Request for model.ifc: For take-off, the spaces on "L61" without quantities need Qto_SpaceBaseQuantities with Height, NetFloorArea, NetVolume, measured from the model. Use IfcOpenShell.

First a look at what the model holds.

```python
import ifcopenshell
import ifcopenshell.util.element
import ifcopenshell.util.unit

model = ifcopenshell.open("model.ifc")
print(model.schema)
for unit_type in ("LENGTHUNIT", "AREAUNIT", "VOLUMEUNIT"):
    print(unit_type, ifcopenshell.util.unit.calculate_unit_scale(model, unit_type))
storey = next(s for s in model.by_type("IfcBuildingStorey") if s.Name == "L61")
spaces = [e for e in ifcopenshell.util.element.get_decomposition(storey) if e.is_a("IfcSpace")]
for e in sorted(spaces, key=lambda e: e.id()):
    print(e.id(), e.is_a(), e.Name, list(ifcopenshell.util.element.get_psets(e, qtos_only=True)), sep=" | ")
```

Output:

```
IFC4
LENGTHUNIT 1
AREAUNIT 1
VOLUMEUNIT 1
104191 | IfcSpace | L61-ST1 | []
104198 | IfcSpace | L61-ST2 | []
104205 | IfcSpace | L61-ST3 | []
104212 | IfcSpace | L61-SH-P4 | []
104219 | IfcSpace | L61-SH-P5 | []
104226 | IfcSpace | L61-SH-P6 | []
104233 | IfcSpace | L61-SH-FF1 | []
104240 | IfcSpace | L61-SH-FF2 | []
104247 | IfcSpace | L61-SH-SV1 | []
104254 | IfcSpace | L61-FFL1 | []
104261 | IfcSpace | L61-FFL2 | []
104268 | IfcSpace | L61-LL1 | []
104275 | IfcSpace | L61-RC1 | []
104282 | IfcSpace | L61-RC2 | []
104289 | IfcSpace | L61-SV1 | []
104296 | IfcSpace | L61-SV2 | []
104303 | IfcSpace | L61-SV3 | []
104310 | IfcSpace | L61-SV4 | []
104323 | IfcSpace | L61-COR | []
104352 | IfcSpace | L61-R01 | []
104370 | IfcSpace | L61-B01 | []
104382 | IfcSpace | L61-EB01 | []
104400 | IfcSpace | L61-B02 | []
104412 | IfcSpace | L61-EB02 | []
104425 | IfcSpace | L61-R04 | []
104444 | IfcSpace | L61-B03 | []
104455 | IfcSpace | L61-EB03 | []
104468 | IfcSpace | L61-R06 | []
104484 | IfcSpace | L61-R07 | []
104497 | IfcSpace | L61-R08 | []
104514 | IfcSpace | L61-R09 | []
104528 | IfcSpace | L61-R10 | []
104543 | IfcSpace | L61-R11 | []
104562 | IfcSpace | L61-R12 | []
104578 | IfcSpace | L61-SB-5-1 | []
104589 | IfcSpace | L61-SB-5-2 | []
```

```python
import ifcopenshell
import ifcopenshell.api.pset
import ifcopenshell.geom
import ifcopenshell.util.element
import ifcopenshell.util.shape
import ifcopenshell.util.unit

model = ifcopenshell.open("model.ifc")
unit_scale = ifcopenshell.util.unit.calculate_unit_scale(model)
area_scale = ifcopenshell.util.unit.calculate_unit_scale(model, "AREAUNIT")
volume_scale = ifcopenshell.util.unit.calculate_unit_scale(model, "VOLUMEUNIT")
settings = ifcopenshell.geom.settings()

storey = next(s for s in model.by_type("IfcBuildingStorey") if s.Name == "L61")
spaces = [e for e in ifcopenshell.util.element.get_decomposition(storey) if e.is_a("IfcSpace")]

for e in sorted(spaces, key=lambda e: e.id()):
    if ifcopenshell.util.element.get_psets(e, qtos_only=True, should_inherit=False):
        continue
    # Geometry comes back in metres, in the element's own axes.
    shape = ifcopenshell.geom.create_shape(settings, e)
    values = {
        "Height": ifcopenshell.util.shape.get_z(shape.geometry) / unit_scale,
        "NetFloorArea": ifcopenshell.util.shape.get_footprint_area(shape.geometry) / area_scale,
        "NetVolume": ifcopenshell.util.shape.get_volume(shape.geometry) / volume_scale,
    }
    qto = ifcopenshell.api.pset.add_qto(model, product=e, name="Qto_SpaceBaseQuantities")
    ifcopenshell.api.pset.edit_qto(model, qto=qto, properties=values)
    print(e.id(), {k: round(v, 3) for k, v in values.items()})

model.write("model_edited.ifc")
```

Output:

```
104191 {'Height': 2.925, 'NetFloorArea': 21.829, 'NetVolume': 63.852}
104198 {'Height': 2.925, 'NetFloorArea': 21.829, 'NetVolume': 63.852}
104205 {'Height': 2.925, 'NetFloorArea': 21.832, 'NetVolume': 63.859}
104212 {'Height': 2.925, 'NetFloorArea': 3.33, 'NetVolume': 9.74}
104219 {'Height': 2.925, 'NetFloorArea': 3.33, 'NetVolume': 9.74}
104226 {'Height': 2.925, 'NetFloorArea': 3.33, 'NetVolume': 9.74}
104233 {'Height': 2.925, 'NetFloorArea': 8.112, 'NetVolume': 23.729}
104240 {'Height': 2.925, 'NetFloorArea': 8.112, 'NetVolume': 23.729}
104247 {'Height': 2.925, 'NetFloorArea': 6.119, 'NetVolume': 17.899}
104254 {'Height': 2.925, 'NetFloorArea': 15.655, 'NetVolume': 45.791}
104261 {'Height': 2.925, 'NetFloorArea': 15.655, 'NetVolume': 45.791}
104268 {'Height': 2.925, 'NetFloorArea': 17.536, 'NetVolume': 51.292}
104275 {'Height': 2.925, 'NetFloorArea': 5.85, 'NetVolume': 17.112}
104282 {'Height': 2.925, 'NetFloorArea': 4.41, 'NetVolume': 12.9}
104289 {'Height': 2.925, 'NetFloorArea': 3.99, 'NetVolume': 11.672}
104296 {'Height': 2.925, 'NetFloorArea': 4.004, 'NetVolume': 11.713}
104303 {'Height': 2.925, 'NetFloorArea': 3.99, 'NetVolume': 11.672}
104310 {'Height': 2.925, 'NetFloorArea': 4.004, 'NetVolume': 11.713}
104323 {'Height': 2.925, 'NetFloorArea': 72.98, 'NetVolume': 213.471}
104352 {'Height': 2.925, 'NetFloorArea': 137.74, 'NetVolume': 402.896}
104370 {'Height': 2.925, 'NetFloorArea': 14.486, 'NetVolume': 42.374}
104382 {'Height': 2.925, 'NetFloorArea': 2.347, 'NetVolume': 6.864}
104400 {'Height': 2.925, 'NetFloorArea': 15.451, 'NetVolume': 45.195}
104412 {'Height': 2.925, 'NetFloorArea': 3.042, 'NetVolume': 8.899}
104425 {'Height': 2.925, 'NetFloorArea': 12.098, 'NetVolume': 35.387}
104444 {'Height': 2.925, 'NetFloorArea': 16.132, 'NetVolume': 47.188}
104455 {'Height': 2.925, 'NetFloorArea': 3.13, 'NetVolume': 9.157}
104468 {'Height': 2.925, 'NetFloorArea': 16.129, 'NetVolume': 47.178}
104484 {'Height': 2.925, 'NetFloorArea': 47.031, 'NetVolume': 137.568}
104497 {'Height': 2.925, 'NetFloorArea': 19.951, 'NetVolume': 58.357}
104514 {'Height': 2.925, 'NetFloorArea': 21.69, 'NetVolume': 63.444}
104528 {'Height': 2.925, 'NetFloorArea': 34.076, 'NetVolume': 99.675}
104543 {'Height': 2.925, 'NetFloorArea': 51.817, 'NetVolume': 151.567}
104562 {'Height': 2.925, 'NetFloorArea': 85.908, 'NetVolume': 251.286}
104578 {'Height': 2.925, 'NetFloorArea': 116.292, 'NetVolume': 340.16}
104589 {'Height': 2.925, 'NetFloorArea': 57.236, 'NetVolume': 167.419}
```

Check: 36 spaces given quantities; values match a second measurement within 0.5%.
